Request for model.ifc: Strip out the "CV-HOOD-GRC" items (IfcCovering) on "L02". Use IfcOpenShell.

First a look at what the model holds.

```python
import ifcopenshell
import ifcopenshell.util.element

model = ifcopenshell.open("model.ifc")
print(model.schema)
storey = next(s for s in model.by_type("IfcBuildingStorey") if s.Name == "L02")
coverings = [e for e in ifcopenshell.util.element.get_decomposition(storey) if e.is_a("IfcCovering")]
seen = {}
for e in coverings:
    element_type = ifcopenshell.util.element.get_type(e)
    name = element_type.Name if element_type not in (None, e) else None
    seen[name] = seen.get(name, 0) + 1
for name, count in sorted(seen.items(), key=str):
    print(count, "x", name)
```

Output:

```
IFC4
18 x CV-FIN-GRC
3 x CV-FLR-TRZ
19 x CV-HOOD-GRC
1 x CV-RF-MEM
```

```python
import ifcopenshell
import ifcopenshell.api.root
import ifcopenshell.util.element

model = ifcopenshell.open("model.ifc")

storey = next(s for s in model.by_type("IfcBuildingStorey") if s.Name == "L02")
coverings = [e for e in ifcopenshell.util.element.get_decomposition(storey) if e.is_a("IfcCovering")]
targets = [e for e in coverings if (t := ifcopenshell.util.element.get_type(e)) not in (None, e) and t.Name == "CV-HOOD-GRC"]

for e in targets:
    ifcopenshell.api.root.remove_product(model, product=e)
print(len(targets), "removed")

model.write("model_updated.ifc")
```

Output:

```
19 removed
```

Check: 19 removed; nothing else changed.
